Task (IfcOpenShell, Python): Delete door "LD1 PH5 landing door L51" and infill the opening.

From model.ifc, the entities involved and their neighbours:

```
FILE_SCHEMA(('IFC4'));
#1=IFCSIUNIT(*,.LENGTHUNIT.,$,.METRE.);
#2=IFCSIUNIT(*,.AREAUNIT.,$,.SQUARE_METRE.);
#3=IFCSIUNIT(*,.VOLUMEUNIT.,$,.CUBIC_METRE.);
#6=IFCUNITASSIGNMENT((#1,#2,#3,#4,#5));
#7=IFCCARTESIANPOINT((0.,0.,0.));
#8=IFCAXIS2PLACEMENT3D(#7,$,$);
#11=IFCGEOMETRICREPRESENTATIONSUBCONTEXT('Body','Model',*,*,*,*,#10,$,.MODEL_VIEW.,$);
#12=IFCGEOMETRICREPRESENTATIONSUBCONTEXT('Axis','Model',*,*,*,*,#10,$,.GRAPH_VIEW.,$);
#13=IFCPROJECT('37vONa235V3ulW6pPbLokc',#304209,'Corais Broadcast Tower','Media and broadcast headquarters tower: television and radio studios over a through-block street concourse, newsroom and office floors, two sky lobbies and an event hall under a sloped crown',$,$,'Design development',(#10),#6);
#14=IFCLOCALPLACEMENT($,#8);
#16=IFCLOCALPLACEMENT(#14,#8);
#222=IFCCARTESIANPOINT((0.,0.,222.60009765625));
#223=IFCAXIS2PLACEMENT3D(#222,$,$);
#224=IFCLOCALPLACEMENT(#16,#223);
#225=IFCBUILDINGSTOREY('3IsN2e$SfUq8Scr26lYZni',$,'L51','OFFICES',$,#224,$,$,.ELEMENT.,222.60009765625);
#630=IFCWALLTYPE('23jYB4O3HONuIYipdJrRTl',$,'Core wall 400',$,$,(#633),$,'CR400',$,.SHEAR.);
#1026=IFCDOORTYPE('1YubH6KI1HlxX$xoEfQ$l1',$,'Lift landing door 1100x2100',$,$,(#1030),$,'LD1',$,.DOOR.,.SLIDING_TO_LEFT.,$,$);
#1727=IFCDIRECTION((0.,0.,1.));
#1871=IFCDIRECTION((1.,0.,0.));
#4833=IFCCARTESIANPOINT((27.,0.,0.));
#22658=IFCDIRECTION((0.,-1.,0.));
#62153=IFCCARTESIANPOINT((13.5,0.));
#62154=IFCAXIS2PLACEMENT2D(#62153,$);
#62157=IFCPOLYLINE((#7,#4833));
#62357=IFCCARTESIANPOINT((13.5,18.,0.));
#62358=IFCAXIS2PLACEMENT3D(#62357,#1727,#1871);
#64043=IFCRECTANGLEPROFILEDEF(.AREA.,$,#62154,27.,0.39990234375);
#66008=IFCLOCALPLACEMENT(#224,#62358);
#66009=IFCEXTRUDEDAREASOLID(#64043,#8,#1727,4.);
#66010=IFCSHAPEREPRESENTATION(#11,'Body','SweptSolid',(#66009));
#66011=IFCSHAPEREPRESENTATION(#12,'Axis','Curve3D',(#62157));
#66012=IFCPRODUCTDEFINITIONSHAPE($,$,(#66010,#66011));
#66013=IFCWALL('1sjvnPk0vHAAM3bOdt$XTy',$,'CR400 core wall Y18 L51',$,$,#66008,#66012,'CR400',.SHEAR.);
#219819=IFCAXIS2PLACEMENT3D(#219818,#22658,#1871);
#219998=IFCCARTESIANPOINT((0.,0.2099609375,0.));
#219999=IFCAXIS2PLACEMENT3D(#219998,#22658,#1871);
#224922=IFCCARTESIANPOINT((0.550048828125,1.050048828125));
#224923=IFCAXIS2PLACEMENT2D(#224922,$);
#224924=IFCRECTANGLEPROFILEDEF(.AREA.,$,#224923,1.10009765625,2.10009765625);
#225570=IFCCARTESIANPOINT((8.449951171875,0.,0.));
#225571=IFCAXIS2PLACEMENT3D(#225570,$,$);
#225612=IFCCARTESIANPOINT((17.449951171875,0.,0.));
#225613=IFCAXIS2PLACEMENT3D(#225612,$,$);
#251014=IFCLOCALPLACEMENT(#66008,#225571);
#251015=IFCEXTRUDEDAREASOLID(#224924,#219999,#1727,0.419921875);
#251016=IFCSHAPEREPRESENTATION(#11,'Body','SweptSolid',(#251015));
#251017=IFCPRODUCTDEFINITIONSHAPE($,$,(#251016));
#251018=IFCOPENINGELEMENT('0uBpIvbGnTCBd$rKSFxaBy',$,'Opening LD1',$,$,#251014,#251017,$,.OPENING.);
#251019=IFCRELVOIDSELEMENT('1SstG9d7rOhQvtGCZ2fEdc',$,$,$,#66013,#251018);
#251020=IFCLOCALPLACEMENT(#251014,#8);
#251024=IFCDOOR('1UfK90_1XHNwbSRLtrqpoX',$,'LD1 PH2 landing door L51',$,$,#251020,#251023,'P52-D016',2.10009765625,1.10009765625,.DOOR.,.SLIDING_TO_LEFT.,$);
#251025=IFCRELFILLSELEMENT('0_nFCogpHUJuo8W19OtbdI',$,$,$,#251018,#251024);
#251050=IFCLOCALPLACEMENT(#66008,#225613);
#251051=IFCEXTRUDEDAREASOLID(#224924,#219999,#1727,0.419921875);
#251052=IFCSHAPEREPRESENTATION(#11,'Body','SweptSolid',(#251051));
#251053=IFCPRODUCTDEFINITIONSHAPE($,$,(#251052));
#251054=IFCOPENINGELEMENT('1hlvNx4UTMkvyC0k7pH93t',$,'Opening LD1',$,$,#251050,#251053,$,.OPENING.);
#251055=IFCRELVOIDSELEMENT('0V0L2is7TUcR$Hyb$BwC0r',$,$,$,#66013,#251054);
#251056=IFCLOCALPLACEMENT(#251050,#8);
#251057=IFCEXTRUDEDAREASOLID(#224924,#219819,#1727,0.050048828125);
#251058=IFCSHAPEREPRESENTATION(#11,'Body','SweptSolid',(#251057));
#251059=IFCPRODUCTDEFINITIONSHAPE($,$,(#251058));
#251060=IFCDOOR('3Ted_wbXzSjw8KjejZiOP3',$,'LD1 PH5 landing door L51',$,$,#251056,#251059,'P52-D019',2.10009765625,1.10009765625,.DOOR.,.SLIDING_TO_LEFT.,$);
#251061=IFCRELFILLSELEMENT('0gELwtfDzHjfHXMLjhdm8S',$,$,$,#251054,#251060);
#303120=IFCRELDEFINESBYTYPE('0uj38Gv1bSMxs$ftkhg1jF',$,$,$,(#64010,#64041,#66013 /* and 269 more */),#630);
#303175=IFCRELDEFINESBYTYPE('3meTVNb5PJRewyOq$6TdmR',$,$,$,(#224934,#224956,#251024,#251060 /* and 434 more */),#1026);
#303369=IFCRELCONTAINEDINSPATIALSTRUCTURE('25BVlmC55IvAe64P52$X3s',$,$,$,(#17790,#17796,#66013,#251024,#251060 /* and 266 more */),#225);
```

```python
import ifcopenshell
import ifcopenshell.api.feature
import ifcopenshell.api.root
import ifcopenshell.geom
import ifcopenshell.util.shape

model = ifcopenshell.open("model.ifc")
settings = ifcopenshell.geom.settings()


def volume(element):
    """Net volume in cubic metres, openings subtracted."""
    shape = ifcopenshell.geom.create_shape(settings, element)
    return ifcopenshell.util.shape.get_volume(shape.geometry)


door = model.by_guid("3Ted_wbXzSjw8KjejZiOP3")
opening = door.FillsVoids[0].RelatingOpeningElement
wall = opening.VoidsElements[0].RelatingBuildingElement
before = volume(wall)

ifcopenshell.api.root.remove_product(model, product=door)
ifcopenshell.api.feature.remove_feature(model, feature=opening)

after = volume(wall)

print(f"wall volume {before:.3f} -> {after:.3f} m3")

model.write("model_edited.ifc")
```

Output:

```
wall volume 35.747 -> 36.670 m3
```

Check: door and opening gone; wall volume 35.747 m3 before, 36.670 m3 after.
